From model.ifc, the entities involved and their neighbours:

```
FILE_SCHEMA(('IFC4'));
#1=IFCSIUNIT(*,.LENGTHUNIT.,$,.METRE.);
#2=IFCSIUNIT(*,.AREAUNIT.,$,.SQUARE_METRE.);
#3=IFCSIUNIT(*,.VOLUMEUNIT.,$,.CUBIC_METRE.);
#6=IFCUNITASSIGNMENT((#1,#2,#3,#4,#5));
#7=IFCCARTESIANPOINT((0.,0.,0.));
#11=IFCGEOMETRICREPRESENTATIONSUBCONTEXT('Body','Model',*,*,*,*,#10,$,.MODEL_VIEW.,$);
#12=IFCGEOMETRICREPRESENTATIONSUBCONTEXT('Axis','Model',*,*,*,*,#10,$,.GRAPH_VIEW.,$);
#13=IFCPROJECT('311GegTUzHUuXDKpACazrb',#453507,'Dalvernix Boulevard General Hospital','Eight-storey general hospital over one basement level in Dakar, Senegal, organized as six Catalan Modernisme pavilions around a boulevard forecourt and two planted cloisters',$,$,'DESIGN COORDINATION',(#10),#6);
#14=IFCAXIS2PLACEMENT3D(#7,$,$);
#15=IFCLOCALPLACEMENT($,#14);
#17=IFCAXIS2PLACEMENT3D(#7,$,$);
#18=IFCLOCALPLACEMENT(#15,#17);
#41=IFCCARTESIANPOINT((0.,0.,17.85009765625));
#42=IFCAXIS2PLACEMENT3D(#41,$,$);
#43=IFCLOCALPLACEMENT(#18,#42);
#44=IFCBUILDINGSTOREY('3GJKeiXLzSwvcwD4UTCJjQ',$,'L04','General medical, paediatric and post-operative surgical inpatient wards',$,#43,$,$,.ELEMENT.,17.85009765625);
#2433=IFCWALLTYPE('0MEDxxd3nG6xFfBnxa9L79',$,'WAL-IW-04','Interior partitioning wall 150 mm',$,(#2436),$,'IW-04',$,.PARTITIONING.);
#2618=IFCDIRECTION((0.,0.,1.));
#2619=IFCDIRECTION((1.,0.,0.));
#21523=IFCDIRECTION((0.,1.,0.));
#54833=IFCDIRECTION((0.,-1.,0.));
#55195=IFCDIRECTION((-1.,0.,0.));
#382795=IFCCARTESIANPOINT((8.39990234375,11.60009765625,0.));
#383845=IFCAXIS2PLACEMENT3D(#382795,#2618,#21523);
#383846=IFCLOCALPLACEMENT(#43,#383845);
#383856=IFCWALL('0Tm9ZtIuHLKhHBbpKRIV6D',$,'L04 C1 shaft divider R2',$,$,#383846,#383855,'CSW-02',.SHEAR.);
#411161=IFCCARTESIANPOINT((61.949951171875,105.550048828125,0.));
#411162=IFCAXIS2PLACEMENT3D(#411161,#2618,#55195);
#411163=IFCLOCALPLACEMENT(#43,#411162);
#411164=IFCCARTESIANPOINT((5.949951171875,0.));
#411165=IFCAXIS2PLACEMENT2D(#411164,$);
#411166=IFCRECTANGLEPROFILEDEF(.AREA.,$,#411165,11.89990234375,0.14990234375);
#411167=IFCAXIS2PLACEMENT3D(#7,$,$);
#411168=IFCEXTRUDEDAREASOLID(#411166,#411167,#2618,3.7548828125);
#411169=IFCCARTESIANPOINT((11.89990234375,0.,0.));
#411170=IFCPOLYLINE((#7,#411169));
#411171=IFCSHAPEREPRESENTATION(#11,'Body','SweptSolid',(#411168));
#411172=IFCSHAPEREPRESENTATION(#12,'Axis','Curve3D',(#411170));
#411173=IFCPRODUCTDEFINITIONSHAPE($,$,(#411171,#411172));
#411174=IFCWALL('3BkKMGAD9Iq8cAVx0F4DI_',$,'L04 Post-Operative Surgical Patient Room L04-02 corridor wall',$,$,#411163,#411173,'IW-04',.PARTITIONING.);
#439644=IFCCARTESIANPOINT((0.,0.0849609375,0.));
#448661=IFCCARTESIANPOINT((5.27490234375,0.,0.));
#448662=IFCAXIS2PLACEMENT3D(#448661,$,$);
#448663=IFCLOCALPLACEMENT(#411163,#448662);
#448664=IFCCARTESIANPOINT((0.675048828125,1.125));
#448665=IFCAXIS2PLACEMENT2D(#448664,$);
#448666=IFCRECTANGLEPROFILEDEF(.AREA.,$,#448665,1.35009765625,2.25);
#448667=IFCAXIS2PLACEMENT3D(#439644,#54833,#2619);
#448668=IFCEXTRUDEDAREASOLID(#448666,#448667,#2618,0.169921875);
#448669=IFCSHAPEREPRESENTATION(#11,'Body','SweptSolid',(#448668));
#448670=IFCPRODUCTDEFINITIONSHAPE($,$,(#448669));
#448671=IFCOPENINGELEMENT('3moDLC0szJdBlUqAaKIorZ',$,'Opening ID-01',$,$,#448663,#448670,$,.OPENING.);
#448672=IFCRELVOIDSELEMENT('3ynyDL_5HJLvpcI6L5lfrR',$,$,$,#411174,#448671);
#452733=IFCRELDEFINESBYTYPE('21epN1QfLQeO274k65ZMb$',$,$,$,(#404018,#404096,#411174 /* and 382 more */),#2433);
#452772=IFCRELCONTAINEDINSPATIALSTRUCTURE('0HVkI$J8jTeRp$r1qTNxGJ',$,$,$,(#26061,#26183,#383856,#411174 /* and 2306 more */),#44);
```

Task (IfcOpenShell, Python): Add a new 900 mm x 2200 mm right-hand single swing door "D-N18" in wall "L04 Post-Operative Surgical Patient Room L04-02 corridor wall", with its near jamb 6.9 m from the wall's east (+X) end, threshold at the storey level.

```python
import numpy as np
import ifcopenshell
import ifcopenshell.api.feature
import ifcopenshell.api.geometry
import ifcopenshell.api.root
import ifcopenshell.api.spatial
import ifcopenshell.geom
import ifcopenshell.util.element
import ifcopenshell.util.placement
import ifcopenshell.util.representation
import ifcopenshell.util.shape
import ifcopenshell.util.unit

model = ifcopenshell.open("model.ifc")
unit_scale = ifcopenshell.util.unit.calculate_unit_scale(model)
settings = ifcopenshell.geom.settings()


def volume(element):
    """Net volume in cubic metres, openings subtracted."""
    shape = ifcopenshell.geom.create_shape(settings, element)
    return ifcopenshell.util.shape.get_volume(shape.geometry)


wall = model.by_guid("3BkKMGAD9Iq8cAVx0F4DI_")
storey = ifcopenshell.util.element.get_container(wall, ifc_class="IfcBuildingStorey")
context = ifcopenshell.util.representation.get_context(model, "Model", "Body", "MODEL_VIEW")
before = volume(wall)

width, height, from_end, sill = 0.9, 2.2, 6.9, 0.0  # metres

# The wall runs along its own X axis, and the end named is its -X end.
wall_shape = ifcopenshell.geom.create_shape(settings, wall)
x, y, z = ifcopenshell.util.shape.get_vertices(wall_shape.geometry).T
start = x.min() + from_end
face, thickness = float(y.min()), float(y.max() - y.min())
wall_matrix = ifcopenshell.util.placement.get_local_placement(wall.ObjectPlacement)
level = ifcopenshell.util.placement.get_local_placement(storey.ObjectPlacement)[2, 3]


def in_wall(x, y):
    """Placement at x, y metres in the wall's axes, at sill height."""
    matrix = wall_matrix.copy()
    matrix[:, 3] = wall_matrix @ np.array([x / unit_scale, y / unit_scale, 0.0, 1.0])
    matrix[2, 3] = level + sill / unit_scale
    return matrix


# Opening: a box that overshoots both wall faces by 50 mm.
opening = ifcopenshell.api.root.create_entity(model, ifc_class="IfcOpeningElement", predefined_type="OPENING")
box = ifcopenshell.api.geometry.add_wall_representation(
    model, context=context, length=width, height=height, thickness=thickness + 0.1
)
ifcopenshell.api.geometry.assign_representation(model, product=opening, representation=box)
ifcopenshell.api.geometry.edit_object_placement(model, product=opening, matrix=in_wall(start, face - 0.05), is_si=False)
ifcopenshell.api.feature.add_feature(model, feature=opening, element=wall)

door = ifcopenshell.api.root.create_entity(model, ifc_class="IfcDoor", name="D-N18", predefined_type="DOOR")
door.OverallWidth, door.OverallHeight = width / unit_scale, height / unit_scale
door.OperationType = "SINGLE_SWING_RIGHT"
body = ifcopenshell.api.geometry.add_door_representation(
    model,
    context=context,
    overall_width=door.OverallWidth,
    overall_height=door.OverallHeight,
    operation_type="SINGLE_SWING_RIGHT",
    lining_properties={"LiningDepth": thickness / unit_scale, "ThresholdDepth": thickness / unit_scale},
)
ifcopenshell.api.geometry.assign_representation(model, product=door, representation=body)
ifcopenshell.api.spatial.assign_container(model, products=[door], relating_structure=storey)
ifcopenshell.api.feature.add_filling(model, opening=opening, element=door)

# The lining spans the wall, so the door starts at the wall face.
ifcopenshell.api.geometry.edit_object_placement(model, product=door, matrix=in_wall(start, face), is_si=False)

after = volume(wall)

print(f"wall volume {before:.3f} -> {after:.3f} m3")

model.write("model_edited.ifc")
```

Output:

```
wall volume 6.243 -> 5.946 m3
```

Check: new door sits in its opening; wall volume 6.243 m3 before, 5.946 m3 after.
